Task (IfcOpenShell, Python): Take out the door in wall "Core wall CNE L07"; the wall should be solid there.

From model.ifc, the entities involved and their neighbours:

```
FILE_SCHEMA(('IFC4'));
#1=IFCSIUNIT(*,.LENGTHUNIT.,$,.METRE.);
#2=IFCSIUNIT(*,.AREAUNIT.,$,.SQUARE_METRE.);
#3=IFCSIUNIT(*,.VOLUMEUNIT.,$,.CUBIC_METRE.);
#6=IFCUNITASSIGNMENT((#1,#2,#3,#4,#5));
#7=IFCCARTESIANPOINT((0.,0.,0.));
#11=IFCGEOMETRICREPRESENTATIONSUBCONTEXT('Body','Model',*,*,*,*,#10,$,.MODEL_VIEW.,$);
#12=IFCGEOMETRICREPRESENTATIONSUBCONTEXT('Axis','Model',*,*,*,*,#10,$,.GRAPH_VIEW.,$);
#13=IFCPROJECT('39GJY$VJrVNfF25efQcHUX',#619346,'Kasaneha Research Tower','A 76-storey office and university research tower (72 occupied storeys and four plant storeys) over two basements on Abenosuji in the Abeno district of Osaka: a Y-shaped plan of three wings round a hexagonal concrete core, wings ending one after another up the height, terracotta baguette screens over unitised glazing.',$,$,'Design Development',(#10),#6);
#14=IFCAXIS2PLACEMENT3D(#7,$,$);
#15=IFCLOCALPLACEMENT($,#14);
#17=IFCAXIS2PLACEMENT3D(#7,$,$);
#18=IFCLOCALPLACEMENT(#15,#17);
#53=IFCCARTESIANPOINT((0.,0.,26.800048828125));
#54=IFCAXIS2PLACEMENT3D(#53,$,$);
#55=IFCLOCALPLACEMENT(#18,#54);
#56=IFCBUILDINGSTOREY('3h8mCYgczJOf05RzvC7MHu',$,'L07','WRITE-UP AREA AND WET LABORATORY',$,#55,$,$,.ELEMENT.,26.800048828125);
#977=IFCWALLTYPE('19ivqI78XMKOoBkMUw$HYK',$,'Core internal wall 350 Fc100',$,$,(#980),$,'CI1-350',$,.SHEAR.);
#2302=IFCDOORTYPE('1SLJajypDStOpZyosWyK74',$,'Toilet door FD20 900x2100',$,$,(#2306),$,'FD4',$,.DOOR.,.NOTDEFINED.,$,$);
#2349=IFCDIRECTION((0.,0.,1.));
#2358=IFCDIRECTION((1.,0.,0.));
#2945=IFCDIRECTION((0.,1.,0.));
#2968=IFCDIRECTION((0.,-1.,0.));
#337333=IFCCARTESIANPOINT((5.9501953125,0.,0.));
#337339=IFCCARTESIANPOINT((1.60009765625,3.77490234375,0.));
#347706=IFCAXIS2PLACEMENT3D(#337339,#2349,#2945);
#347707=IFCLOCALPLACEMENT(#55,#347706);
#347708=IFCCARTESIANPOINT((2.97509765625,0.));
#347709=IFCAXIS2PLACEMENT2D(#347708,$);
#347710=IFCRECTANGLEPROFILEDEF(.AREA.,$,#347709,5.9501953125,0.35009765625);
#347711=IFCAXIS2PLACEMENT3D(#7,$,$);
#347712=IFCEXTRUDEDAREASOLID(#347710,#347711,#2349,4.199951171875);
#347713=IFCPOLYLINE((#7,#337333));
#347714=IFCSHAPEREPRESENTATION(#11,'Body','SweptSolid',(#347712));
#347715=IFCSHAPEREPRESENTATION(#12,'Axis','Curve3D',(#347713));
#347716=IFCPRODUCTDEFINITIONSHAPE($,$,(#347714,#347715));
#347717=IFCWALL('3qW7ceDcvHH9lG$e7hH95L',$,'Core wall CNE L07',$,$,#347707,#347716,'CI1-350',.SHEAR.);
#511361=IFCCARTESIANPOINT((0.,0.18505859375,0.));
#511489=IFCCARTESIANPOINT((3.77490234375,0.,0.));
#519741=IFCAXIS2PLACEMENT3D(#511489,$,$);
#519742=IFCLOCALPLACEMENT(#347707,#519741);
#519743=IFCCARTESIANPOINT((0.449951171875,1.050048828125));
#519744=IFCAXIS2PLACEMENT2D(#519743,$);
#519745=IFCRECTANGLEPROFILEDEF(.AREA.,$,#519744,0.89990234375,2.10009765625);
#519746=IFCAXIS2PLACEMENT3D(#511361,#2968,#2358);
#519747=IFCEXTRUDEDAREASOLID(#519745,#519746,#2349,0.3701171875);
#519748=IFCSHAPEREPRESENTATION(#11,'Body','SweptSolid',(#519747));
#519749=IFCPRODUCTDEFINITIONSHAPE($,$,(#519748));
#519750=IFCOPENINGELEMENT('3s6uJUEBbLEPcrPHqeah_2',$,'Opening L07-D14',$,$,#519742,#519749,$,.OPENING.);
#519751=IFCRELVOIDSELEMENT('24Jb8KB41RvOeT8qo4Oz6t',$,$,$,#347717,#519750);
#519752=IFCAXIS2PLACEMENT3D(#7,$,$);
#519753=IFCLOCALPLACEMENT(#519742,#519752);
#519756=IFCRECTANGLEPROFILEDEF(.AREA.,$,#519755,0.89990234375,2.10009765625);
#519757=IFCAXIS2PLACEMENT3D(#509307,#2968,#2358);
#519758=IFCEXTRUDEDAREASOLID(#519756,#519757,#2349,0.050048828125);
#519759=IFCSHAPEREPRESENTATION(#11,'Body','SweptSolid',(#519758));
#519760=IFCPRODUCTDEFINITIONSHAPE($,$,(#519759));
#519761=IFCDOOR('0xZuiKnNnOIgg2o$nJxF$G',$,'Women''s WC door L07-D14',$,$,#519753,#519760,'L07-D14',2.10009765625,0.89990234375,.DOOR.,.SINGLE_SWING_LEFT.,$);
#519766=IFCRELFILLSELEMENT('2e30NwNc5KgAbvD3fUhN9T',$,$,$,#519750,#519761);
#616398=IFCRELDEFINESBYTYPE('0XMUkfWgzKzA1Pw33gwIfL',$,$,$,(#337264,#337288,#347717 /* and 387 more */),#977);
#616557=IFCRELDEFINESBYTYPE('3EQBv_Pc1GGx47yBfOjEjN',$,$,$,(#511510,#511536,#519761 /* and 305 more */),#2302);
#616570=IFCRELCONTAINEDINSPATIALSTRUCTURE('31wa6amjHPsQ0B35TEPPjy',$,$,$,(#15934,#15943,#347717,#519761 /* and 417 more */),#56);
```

```python
import ifcopenshell
import ifcopenshell.api.feature
import ifcopenshell.api.root
import ifcopenshell.geom
import ifcopenshell.util.shape

model = ifcopenshell.open("model.ifc")
settings = ifcopenshell.geom.settings()


def volume(element):
    """Net volume in cubic metres, openings subtracted."""
    shape = ifcopenshell.geom.create_shape(settings, element)
    return ifcopenshell.util.shape.get_volume(shape.geometry)


door = model.by_id(519761)
opening = door.FillsVoids[0].RelatingOpeningElement
wall = opening.VoidsElements[0].RelatingBuildingElement
before = volume(wall)

ifcopenshell.api.root.remove_product(model, product=door)
ifcopenshell.api.feature.remove_feature(model, feature=opening)

after = volume(wall)

print(f"wall volume {before:.3f} -> {after:.3f} m3")

model.write("model_v2.ifc")
```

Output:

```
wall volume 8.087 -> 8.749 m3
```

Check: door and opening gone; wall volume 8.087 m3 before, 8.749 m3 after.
